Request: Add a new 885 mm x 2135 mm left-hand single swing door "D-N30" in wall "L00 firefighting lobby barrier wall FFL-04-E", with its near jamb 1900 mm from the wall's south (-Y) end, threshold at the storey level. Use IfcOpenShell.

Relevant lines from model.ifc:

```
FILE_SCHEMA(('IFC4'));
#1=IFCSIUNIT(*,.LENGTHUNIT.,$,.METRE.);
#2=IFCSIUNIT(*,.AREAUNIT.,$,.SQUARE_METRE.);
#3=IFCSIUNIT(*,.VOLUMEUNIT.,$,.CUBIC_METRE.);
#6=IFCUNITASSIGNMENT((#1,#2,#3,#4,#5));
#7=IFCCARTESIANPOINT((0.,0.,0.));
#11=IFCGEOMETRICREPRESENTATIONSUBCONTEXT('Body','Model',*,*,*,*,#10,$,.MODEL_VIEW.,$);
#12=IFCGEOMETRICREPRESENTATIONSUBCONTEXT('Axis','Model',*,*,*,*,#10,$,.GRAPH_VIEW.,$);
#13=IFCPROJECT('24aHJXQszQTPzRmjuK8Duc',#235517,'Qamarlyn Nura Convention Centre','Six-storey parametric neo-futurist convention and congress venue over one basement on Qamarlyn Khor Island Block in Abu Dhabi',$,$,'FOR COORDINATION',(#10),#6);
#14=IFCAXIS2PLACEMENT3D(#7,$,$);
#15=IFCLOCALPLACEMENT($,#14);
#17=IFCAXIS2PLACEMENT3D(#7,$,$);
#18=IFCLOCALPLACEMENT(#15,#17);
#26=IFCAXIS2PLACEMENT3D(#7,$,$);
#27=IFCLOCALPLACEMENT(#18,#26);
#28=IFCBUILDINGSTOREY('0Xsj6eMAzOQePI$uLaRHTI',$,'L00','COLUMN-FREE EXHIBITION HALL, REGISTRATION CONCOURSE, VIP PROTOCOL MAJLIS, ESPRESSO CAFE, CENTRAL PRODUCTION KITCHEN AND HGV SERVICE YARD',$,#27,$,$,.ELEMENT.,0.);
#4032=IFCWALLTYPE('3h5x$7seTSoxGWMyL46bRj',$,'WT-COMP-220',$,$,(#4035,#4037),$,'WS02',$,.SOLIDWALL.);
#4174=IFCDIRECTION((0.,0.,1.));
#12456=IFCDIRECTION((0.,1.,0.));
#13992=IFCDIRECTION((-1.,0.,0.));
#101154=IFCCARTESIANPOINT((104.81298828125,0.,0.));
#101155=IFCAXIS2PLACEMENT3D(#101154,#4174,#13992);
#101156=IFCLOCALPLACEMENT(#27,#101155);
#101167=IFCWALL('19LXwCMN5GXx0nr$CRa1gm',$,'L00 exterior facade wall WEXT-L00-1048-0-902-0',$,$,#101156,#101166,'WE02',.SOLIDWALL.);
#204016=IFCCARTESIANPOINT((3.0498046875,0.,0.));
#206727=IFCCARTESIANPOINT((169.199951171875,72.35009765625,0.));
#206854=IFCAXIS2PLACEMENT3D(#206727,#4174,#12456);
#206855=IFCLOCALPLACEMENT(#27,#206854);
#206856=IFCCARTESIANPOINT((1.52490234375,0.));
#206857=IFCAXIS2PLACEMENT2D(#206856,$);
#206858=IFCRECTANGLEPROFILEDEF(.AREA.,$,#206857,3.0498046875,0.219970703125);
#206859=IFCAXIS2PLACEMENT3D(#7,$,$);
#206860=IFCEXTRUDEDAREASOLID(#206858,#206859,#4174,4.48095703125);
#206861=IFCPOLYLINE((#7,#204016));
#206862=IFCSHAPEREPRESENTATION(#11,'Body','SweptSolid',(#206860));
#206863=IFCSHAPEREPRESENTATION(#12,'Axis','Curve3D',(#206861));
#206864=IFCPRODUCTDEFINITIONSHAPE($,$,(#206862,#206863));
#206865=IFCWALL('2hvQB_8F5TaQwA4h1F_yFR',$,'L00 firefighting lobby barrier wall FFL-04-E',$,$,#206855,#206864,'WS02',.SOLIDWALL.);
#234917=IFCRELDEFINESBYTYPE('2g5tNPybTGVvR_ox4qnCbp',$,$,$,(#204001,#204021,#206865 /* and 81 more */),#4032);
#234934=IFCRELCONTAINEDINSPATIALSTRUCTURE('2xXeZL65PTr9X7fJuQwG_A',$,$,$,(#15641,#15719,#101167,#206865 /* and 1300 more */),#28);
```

```python
import numpy as np
import ifcopenshell
import ifcopenshell.api.feature
import ifcopenshell.api.geometry
import ifcopenshell.api.root
import ifcopenshell.api.spatial
import ifcopenshell.geom
import ifcopenshell.util.element
import ifcopenshell.util.placement
import ifcopenshell.util.representation
import ifcopenshell.util.shape
import ifcopenshell.util.unit

model = ifcopenshell.open("model.ifc")
unit_scale = ifcopenshell.util.unit.calculate_unit_scale(model)
settings = ifcopenshell.geom.settings()


def volume(element):
    """Net volume in cubic metres, openings subtracted."""
    shape = ifcopenshell.geom.create_shape(settings, element)
    return ifcopenshell.util.shape.get_volume(shape.geometry)


wall = model.by_id(206865)
storey = ifcopenshell.util.element.get_container(wall, ifc_class="IfcBuildingStorey")
context = ifcopenshell.util.representation.get_context(model, "Model", "Body", "MODEL_VIEW")
before = volume(wall)

width, height, from_end, sill = 0.885, 2.135, 1.9, 0.0  # metres

# The wall runs along its own X axis, and the end named is its -X end.
wall_shape = ifcopenshell.geom.create_shape(settings, wall)
x, y, z = ifcopenshell.util.shape.get_vertices(wall_shape.geometry).T
start = x.min() + from_end
face, thickness = float(y.min()), float(y.max() - y.min())
wall_matrix = ifcopenshell.util.placement.get_local_placement(wall.ObjectPlacement)
level = ifcopenshell.util.placement.get_local_placement(storey.ObjectPlacement)[2, 3]


def in_wall(x, y):
    """Placement at x, y metres in the wall's axes, at sill height."""
    matrix = wall_matrix.copy()
    matrix[:, 3] = wall_matrix @ np.array([x / unit_scale, y / unit_scale, 0.0, 1.0])
    matrix[2, 3] = level + sill / unit_scale
    return matrix


# Opening: a box that overshoots both wall faces by 50 mm.
opening = ifcopenshell.api.root.create_entity(model, ifc_class="IfcOpeningElement", predefined_type="OPENING")
box = ifcopenshell.api.geometry.add_wall_representation(
    model, context=context, length=width, height=height, thickness=thickness + 0.1
)
ifcopenshell.api.geometry.assign_representation(model, product=opening, representation=box)
ifcopenshell.api.geometry.edit_object_placement(model, product=opening, matrix=in_wall(start, face - 0.05), is_si=False)
ifcopenshell.api.feature.add_feature(model, feature=opening, element=wall)

door = ifcopenshell.api.root.create_entity(model, ifc_class="IfcDoor", name="D-N30", predefined_type="DOOR")
door.OverallWidth, door.OverallHeight = width / unit_scale, height / unit_scale
door.OperationType = "SINGLE_SWING_LEFT"
body = ifcopenshell.api.geometry.add_door_representation(
    model,
    context=context,
    overall_width=door.OverallWidth,
    overall_height=door.OverallHeight,
    operation_type="SINGLE_SWING_LEFT",
    lining_properties={"LiningDepth": thickness / unit_scale, "ThresholdDepth": thickness / unit_scale},
)
ifcopenshell.api.geometry.assign_representation(model, product=door, representation=body)
ifcopenshell.api.spatial.assign_container(model, products=[door], relating_structure=storey)
ifcopenshell.api.feature.add_filling(model, opening=opening, element=door)

# The lining spans the wall, so the door starts at the wall face.
ifcopenshell.api.geometry.edit_object_placement(model, product=door, matrix=in_wall(start, face), is_si=False)

after = volume(wall)

print(f"wall volume {before:.3f} -> {after:.3f} m3")

model.write("model_v2.ifc")
```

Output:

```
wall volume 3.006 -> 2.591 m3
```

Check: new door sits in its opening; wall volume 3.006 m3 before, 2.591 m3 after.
